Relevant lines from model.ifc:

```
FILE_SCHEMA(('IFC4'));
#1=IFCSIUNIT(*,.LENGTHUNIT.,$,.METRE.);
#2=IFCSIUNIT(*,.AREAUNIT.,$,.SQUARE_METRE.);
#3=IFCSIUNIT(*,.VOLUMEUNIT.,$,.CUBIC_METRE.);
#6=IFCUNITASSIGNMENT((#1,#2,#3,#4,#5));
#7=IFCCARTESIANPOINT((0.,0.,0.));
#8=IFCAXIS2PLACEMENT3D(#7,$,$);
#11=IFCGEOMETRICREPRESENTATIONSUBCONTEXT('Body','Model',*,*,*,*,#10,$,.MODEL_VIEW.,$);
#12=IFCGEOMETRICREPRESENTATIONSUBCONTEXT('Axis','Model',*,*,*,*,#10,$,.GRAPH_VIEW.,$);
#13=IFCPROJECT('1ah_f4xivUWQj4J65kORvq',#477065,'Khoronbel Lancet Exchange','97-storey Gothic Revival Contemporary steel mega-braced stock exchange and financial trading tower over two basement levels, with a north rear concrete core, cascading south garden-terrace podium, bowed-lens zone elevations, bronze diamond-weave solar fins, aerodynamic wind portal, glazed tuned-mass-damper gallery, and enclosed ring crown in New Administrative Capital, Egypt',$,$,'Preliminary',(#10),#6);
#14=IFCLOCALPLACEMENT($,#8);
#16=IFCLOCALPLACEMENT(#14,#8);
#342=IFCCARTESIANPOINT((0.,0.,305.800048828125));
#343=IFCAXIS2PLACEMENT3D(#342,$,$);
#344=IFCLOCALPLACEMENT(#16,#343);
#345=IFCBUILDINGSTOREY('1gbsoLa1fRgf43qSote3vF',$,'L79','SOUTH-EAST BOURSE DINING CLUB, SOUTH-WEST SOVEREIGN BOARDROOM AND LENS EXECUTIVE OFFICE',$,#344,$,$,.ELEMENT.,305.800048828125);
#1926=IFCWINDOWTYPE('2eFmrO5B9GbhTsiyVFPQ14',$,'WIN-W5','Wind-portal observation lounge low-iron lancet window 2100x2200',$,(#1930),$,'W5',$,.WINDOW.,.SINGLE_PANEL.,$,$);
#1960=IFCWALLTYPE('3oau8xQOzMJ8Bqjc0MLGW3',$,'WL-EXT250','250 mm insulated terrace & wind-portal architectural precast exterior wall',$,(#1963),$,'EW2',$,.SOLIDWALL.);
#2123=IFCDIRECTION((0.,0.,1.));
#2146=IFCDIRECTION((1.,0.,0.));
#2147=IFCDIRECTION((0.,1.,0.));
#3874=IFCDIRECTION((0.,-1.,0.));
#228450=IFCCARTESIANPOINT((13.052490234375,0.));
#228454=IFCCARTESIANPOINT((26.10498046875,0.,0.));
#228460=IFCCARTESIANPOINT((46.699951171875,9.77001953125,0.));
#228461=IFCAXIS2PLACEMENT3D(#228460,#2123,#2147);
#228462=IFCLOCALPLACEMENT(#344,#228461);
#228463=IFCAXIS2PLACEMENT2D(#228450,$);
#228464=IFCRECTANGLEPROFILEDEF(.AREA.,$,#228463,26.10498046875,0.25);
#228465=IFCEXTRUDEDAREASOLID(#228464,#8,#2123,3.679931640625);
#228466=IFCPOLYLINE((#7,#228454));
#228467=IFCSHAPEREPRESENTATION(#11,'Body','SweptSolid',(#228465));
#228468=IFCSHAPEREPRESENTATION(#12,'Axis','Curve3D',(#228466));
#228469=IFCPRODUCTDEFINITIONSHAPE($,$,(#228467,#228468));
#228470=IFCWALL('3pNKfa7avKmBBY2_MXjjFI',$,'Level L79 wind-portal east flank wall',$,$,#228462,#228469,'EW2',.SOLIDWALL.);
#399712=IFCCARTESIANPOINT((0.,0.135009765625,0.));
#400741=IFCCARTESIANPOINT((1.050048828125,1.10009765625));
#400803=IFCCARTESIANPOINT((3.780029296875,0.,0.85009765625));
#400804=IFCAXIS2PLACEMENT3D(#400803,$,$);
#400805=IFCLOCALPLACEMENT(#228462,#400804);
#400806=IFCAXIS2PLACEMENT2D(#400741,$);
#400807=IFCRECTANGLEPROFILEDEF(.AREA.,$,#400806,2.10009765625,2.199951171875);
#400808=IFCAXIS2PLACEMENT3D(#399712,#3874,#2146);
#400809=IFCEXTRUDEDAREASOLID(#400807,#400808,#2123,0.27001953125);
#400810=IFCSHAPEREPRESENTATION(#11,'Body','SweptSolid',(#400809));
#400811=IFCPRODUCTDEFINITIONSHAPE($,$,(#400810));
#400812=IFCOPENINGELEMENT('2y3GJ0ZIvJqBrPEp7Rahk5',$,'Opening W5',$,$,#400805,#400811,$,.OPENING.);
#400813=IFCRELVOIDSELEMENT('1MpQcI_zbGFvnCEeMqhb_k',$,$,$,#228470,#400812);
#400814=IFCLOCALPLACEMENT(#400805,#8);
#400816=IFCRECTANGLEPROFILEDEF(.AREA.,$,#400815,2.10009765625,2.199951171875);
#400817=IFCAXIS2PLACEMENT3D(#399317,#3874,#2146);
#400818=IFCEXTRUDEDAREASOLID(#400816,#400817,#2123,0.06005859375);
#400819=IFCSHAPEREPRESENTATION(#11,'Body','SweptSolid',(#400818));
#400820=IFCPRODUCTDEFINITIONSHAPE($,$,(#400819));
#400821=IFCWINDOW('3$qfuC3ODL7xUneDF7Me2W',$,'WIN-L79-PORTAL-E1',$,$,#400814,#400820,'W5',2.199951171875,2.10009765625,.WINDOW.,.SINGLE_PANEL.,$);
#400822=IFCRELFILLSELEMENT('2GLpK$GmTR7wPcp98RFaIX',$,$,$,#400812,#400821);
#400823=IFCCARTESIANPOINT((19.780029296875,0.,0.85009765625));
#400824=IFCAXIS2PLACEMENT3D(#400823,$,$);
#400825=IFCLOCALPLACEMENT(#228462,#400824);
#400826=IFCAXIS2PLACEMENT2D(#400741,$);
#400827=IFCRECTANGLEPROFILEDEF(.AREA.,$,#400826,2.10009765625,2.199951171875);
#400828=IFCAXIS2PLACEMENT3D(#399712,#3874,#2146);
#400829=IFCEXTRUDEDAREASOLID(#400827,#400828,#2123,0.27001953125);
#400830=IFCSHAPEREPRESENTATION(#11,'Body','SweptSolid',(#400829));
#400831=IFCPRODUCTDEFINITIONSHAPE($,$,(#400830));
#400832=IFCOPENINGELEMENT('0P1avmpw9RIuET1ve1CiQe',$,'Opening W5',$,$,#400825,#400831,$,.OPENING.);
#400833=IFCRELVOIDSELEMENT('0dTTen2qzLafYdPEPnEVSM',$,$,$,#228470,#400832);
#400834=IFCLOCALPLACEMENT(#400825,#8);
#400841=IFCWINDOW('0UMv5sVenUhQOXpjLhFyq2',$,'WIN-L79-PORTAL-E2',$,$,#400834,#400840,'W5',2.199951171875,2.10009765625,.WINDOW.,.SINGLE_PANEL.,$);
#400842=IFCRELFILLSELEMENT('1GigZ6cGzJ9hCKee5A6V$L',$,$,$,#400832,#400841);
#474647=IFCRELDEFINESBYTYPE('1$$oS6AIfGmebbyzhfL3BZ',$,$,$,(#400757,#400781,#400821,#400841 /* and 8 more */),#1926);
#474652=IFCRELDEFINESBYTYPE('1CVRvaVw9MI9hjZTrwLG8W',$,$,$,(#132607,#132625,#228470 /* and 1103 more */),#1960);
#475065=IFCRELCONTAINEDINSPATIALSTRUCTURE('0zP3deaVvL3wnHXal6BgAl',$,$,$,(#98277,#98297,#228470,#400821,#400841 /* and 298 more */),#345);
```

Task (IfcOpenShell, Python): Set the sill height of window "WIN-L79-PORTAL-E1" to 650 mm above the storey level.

```python
import numpy as np
import ifcopenshell
import ifcopenshell.api.geometry
import ifcopenshell.geom
import ifcopenshell.util.element
import ifcopenshell.util.placement
import ifcopenshell.util.shape
import ifcopenshell.util.unit

model = ifcopenshell.open("model.ifc")
unit_scale = ifcopenshell.util.unit.calculate_unit_scale(model)

window = model.by_guid("3$qfuC3ODL7xUneDF7Me2W")
opening = window.FillsVoids[0].RelatingOpeningElement
storey = ifcopenshell.util.element.get_container(window, ifc_class="IfcBuildingStorey")
level = ifcopenshell.util.placement.get_local_placement(storey.ObjectPlacement)[2, 3]

# The opening's origin need not be at the sill, so measure its lowest point.
shape = ifcopenshell.geom.create_shape(ifcopenshell.geom.settings(), opening)
bottom = ifcopenshell.util.shape.get_shape_bottom_elevation(shape, shape.geometry) / unit_scale
dz = level + 0.65 - bottom

shift = np.array([0.0, 0.0, dz])
# The window is placed relative to its opening, so it follows when the opening moves.
matrix = ifcopenshell.util.placement.get_local_placement(opening.ObjectPlacement)
matrix[:3, 3] += shift
ifcopenshell.api.geometry.edit_object_placement(
    model, product=opening, matrix=matrix, is_si=False, should_transform_children=True
)

print(f"moved by {dz * unit_scale:+.3f} m")

model.write("model_rev.ifc")
```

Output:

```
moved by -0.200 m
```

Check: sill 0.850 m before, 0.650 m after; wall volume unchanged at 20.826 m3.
